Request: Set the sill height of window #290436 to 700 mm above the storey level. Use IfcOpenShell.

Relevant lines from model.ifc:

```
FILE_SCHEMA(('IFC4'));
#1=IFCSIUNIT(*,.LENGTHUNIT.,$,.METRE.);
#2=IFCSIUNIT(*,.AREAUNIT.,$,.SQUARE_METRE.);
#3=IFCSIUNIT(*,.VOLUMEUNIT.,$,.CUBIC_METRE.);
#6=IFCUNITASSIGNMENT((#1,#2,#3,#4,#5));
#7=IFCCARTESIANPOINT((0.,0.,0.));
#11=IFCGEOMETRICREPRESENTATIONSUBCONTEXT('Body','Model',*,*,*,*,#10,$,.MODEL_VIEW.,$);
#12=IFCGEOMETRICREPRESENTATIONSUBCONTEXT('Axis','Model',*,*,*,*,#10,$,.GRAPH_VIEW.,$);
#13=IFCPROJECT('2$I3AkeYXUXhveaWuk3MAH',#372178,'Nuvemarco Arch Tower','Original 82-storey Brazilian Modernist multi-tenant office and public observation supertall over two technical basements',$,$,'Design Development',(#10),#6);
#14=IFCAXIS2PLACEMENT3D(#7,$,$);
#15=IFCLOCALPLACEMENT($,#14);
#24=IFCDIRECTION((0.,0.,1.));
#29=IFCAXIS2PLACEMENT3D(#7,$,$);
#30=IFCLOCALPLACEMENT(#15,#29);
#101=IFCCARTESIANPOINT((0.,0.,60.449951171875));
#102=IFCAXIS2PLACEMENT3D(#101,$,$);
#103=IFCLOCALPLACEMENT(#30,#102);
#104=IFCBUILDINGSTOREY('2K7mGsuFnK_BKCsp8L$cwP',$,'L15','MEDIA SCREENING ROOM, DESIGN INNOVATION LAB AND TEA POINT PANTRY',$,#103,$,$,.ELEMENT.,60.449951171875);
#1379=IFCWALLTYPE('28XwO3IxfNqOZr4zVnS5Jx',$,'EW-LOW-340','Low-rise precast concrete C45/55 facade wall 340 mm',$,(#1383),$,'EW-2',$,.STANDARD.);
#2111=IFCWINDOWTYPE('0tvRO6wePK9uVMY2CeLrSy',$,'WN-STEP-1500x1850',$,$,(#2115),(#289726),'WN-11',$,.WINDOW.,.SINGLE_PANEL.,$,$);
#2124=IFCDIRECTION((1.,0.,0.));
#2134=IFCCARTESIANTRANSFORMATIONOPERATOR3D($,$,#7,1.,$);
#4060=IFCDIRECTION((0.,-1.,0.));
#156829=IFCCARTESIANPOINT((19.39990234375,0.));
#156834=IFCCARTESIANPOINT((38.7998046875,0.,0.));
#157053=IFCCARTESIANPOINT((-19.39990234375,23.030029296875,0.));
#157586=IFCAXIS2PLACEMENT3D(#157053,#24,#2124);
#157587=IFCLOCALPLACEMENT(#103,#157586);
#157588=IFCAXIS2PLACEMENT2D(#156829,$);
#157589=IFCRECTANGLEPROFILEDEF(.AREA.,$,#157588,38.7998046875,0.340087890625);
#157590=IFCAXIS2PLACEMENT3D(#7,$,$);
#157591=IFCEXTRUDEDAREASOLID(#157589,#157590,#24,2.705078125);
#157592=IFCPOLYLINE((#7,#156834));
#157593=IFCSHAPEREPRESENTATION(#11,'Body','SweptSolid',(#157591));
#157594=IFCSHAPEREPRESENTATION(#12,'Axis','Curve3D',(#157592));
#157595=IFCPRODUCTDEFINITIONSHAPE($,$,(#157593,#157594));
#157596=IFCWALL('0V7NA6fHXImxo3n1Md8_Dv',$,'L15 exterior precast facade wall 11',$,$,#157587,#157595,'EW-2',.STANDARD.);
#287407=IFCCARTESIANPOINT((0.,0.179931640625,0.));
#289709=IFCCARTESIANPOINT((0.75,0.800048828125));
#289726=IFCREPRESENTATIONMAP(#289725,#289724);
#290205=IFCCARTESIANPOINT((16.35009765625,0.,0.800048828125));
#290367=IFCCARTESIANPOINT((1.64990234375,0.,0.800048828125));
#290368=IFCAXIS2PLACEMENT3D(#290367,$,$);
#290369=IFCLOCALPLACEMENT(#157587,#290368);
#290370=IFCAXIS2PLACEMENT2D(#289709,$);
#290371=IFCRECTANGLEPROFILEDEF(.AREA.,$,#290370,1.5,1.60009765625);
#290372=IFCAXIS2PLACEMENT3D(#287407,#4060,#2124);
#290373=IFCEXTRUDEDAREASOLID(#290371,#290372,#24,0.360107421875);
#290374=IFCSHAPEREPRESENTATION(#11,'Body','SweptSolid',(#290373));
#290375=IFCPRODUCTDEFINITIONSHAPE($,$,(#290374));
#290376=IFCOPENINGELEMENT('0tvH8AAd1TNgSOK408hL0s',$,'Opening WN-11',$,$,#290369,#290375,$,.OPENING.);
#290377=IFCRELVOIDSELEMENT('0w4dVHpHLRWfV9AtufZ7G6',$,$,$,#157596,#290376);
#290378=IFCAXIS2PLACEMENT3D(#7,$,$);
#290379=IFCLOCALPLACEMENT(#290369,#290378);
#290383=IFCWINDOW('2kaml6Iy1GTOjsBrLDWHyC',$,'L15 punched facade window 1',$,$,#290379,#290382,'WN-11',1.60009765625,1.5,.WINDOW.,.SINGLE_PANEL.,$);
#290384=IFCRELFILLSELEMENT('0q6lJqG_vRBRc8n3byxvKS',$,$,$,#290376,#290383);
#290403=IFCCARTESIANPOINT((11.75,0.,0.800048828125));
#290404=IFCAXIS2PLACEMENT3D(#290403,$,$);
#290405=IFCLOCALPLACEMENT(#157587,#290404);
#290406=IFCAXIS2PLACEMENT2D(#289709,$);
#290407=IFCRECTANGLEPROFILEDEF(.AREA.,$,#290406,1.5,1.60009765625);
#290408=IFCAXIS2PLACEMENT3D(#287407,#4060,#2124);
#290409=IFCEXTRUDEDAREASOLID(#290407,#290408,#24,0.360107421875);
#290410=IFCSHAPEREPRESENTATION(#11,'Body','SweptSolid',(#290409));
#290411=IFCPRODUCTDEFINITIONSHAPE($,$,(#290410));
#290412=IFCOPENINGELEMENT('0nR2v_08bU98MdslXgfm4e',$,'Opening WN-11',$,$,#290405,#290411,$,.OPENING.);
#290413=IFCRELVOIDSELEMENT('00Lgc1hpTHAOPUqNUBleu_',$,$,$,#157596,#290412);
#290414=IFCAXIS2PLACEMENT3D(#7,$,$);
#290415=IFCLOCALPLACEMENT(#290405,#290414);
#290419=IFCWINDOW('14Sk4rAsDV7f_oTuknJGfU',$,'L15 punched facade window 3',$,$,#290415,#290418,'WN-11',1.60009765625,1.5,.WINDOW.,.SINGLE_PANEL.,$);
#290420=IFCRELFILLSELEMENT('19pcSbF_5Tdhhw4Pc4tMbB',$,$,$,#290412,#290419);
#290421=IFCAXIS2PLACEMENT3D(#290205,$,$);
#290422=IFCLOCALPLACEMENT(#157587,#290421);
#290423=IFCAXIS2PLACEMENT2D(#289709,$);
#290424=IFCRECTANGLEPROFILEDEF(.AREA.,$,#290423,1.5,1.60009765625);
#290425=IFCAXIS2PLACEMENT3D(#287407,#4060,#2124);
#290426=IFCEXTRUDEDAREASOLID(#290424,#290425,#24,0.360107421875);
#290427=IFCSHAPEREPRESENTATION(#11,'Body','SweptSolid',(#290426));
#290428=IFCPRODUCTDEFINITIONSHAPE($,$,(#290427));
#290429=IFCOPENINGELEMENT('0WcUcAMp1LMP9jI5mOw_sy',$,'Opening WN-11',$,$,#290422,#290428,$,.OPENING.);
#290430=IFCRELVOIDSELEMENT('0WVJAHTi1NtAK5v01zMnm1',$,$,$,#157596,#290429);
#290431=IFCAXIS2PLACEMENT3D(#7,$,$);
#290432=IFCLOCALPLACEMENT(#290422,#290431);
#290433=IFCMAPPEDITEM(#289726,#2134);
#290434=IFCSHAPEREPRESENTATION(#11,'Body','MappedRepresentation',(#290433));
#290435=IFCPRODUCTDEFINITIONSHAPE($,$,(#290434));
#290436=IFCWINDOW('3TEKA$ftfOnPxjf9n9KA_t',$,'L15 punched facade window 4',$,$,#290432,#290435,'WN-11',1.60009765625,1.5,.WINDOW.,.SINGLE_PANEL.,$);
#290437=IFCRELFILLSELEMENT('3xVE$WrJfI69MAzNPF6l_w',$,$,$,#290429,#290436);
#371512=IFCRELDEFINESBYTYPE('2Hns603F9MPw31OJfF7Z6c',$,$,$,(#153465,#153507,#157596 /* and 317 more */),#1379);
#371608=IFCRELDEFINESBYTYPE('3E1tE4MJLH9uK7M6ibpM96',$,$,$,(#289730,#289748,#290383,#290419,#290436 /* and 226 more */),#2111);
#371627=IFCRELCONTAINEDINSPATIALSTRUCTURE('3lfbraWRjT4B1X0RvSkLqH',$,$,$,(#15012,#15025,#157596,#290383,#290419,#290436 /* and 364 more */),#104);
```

```python
import numpy as np
import ifcopenshell
import ifcopenshell.api.geometry
import ifcopenshell.geom
import ifcopenshell.util.element
import ifcopenshell.util.placement
import ifcopenshell.util.shape
import ifcopenshell.util.unit

model = ifcopenshell.open("model.ifc")
unit_scale = ifcopenshell.util.unit.calculate_unit_scale(model)

window = model.by_id(290436)
opening = window.FillsVoids[0].RelatingOpeningElement
storey = ifcopenshell.util.element.get_container(window, ifc_class="IfcBuildingStorey")
level = ifcopenshell.util.placement.get_local_placement(storey.ObjectPlacement)[2, 3]

# The opening's origin need not be at the sill, so measure its lowest point.
shape = ifcopenshell.geom.create_shape(ifcopenshell.geom.settings(), opening)
bottom = ifcopenshell.util.shape.get_shape_bottom_elevation(shape, shape.geometry) / unit_scale
dz = level + 0.7 / unit_scale - bottom

shift = np.array([0.0, 0.0, dz])
# The window is placed relative to its opening, so it follows when the opening moves.
matrix = ifcopenshell.util.placement.get_local_placement(opening.ObjectPlacement)
matrix[:3, 3] += shift
ifcopenshell.api.geometry.edit_object_placement(
    model, product=opening, matrix=matrix, is_si=False, should_transform_children=True
)

print(f"moved by {dz * unit_scale:+.3f} m")

model.write("model_rev.ifc")
```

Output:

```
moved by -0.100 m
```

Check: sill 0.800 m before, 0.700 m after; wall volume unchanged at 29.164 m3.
